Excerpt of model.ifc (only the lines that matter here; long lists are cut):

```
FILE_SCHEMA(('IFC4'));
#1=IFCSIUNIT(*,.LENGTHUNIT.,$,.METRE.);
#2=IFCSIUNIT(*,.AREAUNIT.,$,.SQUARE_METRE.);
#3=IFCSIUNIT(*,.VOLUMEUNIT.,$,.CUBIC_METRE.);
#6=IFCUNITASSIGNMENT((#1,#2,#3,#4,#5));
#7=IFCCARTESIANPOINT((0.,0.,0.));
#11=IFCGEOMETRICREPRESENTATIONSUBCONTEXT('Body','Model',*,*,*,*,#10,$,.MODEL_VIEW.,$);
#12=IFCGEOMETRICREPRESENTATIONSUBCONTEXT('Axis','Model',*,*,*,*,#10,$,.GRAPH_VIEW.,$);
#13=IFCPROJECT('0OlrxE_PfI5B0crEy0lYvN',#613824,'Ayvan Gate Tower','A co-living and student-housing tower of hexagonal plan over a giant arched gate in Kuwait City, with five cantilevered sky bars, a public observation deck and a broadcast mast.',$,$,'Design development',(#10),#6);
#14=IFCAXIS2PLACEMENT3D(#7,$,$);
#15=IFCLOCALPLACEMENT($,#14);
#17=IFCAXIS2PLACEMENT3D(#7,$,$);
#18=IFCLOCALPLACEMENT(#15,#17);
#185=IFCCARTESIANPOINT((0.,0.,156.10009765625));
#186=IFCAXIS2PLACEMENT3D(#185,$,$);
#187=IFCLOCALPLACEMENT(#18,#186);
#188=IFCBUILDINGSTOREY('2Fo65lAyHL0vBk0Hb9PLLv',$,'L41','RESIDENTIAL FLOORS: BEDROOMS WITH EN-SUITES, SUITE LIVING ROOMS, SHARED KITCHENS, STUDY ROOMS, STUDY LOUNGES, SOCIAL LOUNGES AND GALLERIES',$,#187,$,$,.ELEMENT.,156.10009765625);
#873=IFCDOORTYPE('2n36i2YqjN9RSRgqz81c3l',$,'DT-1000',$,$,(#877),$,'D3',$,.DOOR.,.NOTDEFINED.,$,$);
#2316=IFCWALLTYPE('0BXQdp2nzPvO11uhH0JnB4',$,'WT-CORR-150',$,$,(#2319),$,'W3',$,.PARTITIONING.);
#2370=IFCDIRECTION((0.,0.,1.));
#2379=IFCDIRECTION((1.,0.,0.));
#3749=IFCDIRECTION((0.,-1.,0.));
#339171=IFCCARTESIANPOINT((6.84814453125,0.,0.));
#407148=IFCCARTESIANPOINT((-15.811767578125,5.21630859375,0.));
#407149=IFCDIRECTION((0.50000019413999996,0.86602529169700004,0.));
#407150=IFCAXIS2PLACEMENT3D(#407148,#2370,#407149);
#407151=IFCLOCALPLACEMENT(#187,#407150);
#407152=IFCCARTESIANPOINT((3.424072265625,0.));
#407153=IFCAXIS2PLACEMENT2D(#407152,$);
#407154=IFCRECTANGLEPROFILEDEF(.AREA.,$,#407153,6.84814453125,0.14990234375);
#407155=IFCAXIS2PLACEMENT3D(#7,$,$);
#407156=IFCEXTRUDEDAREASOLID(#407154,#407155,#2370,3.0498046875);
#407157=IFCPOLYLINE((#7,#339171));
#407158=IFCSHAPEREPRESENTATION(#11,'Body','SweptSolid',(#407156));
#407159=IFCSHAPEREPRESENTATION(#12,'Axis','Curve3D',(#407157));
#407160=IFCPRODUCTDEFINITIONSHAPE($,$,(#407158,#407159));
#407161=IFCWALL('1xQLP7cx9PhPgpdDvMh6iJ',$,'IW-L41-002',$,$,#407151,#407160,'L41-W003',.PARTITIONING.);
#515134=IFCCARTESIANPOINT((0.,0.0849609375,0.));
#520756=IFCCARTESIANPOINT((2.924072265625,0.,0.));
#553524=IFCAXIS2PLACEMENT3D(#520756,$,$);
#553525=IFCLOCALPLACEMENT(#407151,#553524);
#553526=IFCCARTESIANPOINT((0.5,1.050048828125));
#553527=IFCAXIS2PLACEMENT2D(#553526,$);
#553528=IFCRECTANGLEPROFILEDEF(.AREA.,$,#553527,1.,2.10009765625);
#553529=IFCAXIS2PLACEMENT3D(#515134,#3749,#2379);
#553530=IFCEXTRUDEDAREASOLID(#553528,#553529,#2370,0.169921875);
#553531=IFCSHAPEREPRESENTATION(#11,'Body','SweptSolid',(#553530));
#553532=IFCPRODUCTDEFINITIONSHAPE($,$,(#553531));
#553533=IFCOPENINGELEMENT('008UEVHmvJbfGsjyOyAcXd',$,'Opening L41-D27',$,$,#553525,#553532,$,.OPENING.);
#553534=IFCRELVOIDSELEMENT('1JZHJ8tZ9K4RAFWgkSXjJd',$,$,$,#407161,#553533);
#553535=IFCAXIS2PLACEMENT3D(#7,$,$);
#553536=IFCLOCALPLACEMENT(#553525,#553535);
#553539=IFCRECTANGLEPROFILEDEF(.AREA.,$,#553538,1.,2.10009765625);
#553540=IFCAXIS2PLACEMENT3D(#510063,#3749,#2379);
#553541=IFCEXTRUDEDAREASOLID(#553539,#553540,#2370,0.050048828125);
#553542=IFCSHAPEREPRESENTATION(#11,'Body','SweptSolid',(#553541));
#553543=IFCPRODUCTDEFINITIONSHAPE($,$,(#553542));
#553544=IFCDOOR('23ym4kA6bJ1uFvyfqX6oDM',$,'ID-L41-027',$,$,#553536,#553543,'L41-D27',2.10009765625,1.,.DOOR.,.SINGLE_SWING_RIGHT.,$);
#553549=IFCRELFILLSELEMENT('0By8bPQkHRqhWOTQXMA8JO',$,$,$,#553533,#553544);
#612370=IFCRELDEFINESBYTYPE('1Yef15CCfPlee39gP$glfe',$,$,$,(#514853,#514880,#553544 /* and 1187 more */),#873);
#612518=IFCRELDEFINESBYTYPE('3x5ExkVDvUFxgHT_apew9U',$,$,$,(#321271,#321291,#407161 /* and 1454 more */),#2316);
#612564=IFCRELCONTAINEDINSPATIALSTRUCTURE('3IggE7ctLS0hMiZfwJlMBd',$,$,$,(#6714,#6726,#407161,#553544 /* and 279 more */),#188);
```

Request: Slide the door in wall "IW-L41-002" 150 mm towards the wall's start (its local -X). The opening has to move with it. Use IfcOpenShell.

```python
import ifcopenshell
import ifcopenshell.api.geometry
import ifcopenshell.util.placement

model = ifcopenshell.open("model.ifc")

door = model.by_id(553544)
opening = door.FillsVoids[0].RelatingOpeningElement
wall = opening.VoidsElements[0].RelatingBuildingElement

wall_matrix = ifcopenshell.util.placement.get_local_placement(wall.ObjectPlacement)
shift = wall_matrix[:3, 0] * -0.15
before = ifcopenshell.util.placement.get_local_placement(door.ObjectPlacement)[:3, 3].copy()

# The door is placed relative to its opening, so it follows when the opening moves.
matrix = ifcopenshell.util.placement.get_local_placement(opening.ObjectPlacement)
matrix[:3, 3] += shift
ifcopenshell.api.geometry.edit_object_placement(
    model, product=opening, matrix=matrix, is_si=False, should_transform_children=True
)

after = ifcopenshell.util.placement.get_local_placement(door.ObjectPlacement)[:3, 3]
print("door moved by", (after - before).round(3) + 0.0)

model.write("model_v2.ifc")
```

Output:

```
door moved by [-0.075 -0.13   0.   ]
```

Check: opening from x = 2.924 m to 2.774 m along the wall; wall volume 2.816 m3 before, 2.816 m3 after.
